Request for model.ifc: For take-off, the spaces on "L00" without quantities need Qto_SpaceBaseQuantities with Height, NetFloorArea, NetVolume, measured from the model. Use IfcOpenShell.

First a look at what the model holds.

```python
import ifcopenshell
import ifcopenshell.util.element
import ifcopenshell.util.unit

model = ifcopenshell.open("model.ifc")
print(model.schema)
for unit_type in ("LENGTHUNIT", "AREAUNIT", "VOLUMEUNIT"):
    print(unit_type, ifcopenshell.util.unit.calculate_unit_scale(model, unit_type))
storey = next(s for s in model.by_type("IfcBuildingStorey") if s.Name == "L00")
spaces = [e for e in ifcopenshell.util.element.get_decomposition(storey) if e.is_a("IfcSpace")]
for e in sorted(spaces, key=lambda e: e.id()):
    print(e.id(), e.is_a(), e.Name, list(ifcopenshell.util.element.get_psets(e, qtos_only=True)), sep=" | ")
```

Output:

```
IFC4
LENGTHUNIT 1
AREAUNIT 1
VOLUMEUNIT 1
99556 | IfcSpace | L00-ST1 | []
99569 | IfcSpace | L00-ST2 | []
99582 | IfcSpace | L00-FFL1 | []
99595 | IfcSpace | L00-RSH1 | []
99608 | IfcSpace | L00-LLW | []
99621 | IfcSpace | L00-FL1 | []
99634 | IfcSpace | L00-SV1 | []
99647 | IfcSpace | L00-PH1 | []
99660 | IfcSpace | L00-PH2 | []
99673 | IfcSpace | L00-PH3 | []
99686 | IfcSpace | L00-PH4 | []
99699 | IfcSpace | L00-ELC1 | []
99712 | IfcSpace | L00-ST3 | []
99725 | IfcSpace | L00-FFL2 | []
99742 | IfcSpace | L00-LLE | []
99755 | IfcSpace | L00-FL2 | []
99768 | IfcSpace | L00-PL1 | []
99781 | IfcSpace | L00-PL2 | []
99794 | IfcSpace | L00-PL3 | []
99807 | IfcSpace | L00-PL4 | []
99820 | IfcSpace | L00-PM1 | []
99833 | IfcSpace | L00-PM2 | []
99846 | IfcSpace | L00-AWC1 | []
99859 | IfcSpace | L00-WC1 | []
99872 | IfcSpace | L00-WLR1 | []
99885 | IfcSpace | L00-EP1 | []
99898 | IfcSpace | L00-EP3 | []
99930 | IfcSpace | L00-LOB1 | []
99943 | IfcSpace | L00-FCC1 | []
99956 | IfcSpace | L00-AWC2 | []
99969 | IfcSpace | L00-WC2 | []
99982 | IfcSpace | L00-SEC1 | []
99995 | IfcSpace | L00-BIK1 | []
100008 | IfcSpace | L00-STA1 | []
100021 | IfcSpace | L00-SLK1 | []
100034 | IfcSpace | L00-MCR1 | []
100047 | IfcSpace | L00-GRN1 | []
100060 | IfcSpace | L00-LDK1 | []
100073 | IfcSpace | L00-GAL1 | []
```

```python
import ifcopenshell
import ifcopenshell.api.pset
import ifcopenshell.geom
import ifcopenshell.util.element
import ifcopenshell.util.shape
import ifcopenshell.util.unit

model = ifcopenshell.open("model.ifc")
unit_scale = ifcopenshell.util.unit.calculate_unit_scale(model)
area_scale = ifcopenshell.util.unit.calculate_unit_scale(model, "AREAUNIT")
volume_scale = ifcopenshell.util.unit.calculate_unit_scale(model, "VOLUMEUNIT")
settings = ifcopenshell.geom.settings()

storey = next(s for s in model.by_type("IfcBuildingStorey") if s.Name == "L00")
spaces = [e for e in ifcopenshell.util.element.get_decomposition(storey) if e.is_a("IfcSpace")]

for e in sorted(spaces, key=lambda e: e.id()):
    if ifcopenshell.util.element.get_psets(e, qtos_only=True, should_inherit=False):
        continue
    # Geometry comes back in metres, in the element's own axes.
    shape = ifcopenshell.geom.create_shape(settings, e)
    values = {
        "Height": ifcopenshell.util.shape.get_z(shape.geometry) / unit_scale,
        "NetFloorArea": ifcopenshell.util.shape.get_footprint_area(shape.geometry) / area_scale,
        "NetVolume": ifcopenshell.util.shape.get_volume(shape.geometry) / volume_scale,
    }
    qto = ifcopenshell.api.pset.add_qto(model, product=e, name="Qto_SpaceBaseQuantities")
    ifcopenshell.api.pset.edit_qto(model, qto=qto, properties=values)
    print(e.id(), {k: round(v, 3) for k, v in values.items()})

model.write("model_rev.ifc")
```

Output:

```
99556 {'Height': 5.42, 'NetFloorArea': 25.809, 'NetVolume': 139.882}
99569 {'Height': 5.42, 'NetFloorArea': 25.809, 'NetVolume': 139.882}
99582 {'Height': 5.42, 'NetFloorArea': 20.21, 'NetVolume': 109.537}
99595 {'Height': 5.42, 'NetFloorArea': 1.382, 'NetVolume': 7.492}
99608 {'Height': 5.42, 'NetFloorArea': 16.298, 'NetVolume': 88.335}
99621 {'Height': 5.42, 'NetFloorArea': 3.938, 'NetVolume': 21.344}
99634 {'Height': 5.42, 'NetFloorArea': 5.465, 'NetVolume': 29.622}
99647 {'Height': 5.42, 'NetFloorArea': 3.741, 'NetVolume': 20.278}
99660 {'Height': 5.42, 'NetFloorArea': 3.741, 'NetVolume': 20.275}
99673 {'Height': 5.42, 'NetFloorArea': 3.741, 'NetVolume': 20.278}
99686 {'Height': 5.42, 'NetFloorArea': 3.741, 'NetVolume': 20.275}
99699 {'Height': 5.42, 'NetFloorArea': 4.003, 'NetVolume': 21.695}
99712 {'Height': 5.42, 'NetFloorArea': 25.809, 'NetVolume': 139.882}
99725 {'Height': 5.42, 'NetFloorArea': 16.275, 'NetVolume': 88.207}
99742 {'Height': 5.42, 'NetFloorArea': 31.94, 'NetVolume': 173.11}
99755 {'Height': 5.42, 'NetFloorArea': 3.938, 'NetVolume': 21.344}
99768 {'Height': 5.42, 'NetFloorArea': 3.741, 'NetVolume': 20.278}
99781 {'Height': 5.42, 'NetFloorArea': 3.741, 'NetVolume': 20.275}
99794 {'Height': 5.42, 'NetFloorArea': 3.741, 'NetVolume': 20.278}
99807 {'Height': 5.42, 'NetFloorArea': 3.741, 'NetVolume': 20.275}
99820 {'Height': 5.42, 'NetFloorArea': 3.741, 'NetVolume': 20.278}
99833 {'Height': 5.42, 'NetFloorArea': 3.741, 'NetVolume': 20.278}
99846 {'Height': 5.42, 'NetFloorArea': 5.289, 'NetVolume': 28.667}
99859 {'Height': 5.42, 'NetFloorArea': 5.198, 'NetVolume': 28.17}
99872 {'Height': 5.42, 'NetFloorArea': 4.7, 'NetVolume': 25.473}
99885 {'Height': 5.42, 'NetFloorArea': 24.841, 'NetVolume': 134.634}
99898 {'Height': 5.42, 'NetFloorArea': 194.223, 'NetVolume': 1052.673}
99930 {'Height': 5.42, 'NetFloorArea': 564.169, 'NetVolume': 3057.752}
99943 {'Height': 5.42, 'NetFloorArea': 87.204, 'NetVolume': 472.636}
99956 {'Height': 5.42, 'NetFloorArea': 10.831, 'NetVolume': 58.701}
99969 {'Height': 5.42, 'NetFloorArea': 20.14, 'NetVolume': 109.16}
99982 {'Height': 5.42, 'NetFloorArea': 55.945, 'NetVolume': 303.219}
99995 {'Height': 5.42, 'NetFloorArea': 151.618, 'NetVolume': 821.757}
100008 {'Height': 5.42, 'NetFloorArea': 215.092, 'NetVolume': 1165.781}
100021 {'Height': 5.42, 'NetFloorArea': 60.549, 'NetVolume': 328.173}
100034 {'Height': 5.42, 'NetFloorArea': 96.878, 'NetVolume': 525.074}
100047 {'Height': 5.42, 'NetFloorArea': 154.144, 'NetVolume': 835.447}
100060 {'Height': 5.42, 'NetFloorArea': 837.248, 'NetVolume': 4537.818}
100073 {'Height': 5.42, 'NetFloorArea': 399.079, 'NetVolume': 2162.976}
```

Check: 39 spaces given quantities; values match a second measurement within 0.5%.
